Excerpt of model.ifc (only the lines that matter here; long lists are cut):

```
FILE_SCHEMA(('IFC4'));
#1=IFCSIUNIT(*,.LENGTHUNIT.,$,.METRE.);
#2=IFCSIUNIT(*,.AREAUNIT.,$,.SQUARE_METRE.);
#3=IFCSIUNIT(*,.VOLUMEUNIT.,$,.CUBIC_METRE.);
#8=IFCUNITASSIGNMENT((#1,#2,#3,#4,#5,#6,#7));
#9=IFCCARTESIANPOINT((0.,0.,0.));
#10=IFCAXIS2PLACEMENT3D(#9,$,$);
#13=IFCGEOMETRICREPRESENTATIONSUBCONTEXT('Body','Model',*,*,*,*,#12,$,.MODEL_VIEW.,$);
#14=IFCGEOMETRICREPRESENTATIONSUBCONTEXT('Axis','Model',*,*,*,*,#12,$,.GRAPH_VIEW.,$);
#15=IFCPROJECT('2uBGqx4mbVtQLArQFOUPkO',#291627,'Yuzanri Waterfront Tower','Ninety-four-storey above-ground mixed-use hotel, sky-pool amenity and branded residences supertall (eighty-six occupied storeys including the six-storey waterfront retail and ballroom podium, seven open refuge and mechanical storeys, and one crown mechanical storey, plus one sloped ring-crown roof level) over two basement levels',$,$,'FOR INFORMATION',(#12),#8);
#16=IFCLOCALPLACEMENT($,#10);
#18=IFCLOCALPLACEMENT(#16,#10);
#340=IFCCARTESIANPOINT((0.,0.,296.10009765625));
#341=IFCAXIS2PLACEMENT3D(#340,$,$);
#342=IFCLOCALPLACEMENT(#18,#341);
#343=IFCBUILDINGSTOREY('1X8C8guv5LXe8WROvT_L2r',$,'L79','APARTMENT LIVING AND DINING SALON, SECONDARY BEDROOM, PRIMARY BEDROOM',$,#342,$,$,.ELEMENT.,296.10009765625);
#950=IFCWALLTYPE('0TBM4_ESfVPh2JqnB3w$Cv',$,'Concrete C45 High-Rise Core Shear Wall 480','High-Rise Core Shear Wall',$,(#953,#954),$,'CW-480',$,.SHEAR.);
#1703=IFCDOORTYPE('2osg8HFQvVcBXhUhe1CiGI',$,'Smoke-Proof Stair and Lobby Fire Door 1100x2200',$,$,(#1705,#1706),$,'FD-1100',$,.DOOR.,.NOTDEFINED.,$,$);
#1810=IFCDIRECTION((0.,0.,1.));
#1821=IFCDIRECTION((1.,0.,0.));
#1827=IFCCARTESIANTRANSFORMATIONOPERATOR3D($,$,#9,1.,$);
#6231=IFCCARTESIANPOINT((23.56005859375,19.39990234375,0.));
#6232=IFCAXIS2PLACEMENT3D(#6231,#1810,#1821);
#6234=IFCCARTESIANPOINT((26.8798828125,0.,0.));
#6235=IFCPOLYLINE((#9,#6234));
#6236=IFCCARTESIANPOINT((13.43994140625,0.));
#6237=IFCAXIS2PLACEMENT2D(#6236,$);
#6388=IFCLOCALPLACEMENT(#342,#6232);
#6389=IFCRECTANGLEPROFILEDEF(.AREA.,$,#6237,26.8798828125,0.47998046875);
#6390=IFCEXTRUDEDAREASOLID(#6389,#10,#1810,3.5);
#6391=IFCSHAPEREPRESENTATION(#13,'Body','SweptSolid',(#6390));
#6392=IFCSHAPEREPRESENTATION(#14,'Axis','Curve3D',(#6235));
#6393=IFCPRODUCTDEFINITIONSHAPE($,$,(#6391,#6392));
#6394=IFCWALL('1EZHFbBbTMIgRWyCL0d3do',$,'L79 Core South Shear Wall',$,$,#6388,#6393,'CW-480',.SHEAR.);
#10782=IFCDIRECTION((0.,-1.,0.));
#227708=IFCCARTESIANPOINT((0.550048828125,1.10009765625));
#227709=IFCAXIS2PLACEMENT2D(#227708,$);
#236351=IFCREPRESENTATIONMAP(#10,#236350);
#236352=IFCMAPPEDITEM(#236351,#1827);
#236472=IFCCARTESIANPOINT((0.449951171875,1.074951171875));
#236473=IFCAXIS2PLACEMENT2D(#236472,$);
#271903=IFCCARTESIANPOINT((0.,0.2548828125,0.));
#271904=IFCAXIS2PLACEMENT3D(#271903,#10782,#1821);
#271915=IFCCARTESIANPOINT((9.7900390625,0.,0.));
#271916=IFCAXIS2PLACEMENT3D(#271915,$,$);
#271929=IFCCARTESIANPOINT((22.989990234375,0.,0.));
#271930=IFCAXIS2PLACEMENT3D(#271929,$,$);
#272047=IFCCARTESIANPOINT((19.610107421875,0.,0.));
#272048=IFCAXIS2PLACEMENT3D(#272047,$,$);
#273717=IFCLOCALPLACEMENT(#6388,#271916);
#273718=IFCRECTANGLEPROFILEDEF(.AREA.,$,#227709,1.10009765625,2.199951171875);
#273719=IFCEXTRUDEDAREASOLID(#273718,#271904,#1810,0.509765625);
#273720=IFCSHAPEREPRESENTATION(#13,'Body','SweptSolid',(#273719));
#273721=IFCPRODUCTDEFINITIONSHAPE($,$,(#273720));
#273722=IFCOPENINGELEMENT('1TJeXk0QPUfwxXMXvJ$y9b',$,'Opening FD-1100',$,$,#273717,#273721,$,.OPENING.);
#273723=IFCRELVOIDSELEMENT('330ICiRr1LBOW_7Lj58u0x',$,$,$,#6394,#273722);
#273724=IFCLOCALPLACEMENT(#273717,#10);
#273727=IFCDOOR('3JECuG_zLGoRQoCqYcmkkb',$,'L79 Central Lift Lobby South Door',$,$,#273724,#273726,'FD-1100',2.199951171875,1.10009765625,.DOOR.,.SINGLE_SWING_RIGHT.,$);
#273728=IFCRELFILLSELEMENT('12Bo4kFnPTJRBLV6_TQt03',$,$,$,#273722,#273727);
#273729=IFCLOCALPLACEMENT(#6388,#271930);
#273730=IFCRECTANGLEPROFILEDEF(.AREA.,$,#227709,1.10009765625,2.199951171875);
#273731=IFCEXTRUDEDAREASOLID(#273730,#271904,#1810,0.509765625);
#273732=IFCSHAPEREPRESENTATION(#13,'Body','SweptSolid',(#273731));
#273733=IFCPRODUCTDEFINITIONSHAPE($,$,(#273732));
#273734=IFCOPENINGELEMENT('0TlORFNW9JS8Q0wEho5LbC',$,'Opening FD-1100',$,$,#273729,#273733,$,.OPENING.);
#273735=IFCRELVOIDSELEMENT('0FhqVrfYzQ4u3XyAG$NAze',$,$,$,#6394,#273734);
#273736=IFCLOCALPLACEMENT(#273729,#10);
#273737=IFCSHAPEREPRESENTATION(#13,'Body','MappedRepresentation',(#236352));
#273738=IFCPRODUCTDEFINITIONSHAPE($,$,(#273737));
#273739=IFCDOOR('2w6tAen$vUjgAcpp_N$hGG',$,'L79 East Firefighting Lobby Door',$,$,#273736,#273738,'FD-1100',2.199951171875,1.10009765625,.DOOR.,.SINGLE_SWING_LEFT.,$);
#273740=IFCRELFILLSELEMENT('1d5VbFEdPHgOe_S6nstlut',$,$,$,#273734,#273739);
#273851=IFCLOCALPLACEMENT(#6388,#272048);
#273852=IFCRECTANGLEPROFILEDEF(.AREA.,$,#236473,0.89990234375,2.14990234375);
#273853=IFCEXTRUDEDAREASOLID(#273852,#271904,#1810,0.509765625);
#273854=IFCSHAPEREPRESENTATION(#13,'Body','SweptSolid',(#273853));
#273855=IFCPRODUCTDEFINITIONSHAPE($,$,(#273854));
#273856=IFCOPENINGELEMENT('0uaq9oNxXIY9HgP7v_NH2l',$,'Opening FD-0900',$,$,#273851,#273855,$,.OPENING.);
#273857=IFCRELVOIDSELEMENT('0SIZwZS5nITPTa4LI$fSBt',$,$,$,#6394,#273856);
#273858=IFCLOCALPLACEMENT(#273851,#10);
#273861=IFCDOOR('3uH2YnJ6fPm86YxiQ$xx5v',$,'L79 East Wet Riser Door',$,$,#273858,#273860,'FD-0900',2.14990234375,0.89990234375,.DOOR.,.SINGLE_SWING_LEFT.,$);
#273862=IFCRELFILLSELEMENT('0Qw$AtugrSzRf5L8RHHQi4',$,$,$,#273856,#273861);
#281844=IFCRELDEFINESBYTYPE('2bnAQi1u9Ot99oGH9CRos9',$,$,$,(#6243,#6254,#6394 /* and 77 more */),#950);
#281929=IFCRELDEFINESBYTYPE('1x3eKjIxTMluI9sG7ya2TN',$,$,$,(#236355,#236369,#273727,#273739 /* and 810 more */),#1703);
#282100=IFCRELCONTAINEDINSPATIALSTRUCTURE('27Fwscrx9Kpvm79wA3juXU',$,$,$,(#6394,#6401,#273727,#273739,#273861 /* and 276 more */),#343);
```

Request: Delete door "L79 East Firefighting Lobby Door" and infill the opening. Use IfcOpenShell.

```python
import ifcopenshell
import ifcopenshell.api.feature
import ifcopenshell.api.root
import ifcopenshell.geom
import ifcopenshell.util.shape

model = ifcopenshell.open("model.ifc")
settings = ifcopenshell.geom.settings()


def volume(element):
    """Net volume in cubic metres, openings subtracted."""
    shape = ifcopenshell.geom.create_shape(settings, element)
    return ifcopenshell.util.shape.get_volume(shape.geometry)


door = model.by_id(273739)
opening = door.FillsVoids[0].RelatingOpeningElement
wall = opening.VoidsElements[0].RelatingBuildingElement
before = volume(wall)

ifcopenshell.api.root.remove_product(model, product=door)
ifcopenshell.api.feature.remove_feature(model, feature=opening)

after = volume(wall)

print(f"wall volume {before:.3f} -> {after:.3f} m3")

model.write("model_updated.ifc")
```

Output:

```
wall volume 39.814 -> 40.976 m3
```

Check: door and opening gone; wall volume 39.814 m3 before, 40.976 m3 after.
